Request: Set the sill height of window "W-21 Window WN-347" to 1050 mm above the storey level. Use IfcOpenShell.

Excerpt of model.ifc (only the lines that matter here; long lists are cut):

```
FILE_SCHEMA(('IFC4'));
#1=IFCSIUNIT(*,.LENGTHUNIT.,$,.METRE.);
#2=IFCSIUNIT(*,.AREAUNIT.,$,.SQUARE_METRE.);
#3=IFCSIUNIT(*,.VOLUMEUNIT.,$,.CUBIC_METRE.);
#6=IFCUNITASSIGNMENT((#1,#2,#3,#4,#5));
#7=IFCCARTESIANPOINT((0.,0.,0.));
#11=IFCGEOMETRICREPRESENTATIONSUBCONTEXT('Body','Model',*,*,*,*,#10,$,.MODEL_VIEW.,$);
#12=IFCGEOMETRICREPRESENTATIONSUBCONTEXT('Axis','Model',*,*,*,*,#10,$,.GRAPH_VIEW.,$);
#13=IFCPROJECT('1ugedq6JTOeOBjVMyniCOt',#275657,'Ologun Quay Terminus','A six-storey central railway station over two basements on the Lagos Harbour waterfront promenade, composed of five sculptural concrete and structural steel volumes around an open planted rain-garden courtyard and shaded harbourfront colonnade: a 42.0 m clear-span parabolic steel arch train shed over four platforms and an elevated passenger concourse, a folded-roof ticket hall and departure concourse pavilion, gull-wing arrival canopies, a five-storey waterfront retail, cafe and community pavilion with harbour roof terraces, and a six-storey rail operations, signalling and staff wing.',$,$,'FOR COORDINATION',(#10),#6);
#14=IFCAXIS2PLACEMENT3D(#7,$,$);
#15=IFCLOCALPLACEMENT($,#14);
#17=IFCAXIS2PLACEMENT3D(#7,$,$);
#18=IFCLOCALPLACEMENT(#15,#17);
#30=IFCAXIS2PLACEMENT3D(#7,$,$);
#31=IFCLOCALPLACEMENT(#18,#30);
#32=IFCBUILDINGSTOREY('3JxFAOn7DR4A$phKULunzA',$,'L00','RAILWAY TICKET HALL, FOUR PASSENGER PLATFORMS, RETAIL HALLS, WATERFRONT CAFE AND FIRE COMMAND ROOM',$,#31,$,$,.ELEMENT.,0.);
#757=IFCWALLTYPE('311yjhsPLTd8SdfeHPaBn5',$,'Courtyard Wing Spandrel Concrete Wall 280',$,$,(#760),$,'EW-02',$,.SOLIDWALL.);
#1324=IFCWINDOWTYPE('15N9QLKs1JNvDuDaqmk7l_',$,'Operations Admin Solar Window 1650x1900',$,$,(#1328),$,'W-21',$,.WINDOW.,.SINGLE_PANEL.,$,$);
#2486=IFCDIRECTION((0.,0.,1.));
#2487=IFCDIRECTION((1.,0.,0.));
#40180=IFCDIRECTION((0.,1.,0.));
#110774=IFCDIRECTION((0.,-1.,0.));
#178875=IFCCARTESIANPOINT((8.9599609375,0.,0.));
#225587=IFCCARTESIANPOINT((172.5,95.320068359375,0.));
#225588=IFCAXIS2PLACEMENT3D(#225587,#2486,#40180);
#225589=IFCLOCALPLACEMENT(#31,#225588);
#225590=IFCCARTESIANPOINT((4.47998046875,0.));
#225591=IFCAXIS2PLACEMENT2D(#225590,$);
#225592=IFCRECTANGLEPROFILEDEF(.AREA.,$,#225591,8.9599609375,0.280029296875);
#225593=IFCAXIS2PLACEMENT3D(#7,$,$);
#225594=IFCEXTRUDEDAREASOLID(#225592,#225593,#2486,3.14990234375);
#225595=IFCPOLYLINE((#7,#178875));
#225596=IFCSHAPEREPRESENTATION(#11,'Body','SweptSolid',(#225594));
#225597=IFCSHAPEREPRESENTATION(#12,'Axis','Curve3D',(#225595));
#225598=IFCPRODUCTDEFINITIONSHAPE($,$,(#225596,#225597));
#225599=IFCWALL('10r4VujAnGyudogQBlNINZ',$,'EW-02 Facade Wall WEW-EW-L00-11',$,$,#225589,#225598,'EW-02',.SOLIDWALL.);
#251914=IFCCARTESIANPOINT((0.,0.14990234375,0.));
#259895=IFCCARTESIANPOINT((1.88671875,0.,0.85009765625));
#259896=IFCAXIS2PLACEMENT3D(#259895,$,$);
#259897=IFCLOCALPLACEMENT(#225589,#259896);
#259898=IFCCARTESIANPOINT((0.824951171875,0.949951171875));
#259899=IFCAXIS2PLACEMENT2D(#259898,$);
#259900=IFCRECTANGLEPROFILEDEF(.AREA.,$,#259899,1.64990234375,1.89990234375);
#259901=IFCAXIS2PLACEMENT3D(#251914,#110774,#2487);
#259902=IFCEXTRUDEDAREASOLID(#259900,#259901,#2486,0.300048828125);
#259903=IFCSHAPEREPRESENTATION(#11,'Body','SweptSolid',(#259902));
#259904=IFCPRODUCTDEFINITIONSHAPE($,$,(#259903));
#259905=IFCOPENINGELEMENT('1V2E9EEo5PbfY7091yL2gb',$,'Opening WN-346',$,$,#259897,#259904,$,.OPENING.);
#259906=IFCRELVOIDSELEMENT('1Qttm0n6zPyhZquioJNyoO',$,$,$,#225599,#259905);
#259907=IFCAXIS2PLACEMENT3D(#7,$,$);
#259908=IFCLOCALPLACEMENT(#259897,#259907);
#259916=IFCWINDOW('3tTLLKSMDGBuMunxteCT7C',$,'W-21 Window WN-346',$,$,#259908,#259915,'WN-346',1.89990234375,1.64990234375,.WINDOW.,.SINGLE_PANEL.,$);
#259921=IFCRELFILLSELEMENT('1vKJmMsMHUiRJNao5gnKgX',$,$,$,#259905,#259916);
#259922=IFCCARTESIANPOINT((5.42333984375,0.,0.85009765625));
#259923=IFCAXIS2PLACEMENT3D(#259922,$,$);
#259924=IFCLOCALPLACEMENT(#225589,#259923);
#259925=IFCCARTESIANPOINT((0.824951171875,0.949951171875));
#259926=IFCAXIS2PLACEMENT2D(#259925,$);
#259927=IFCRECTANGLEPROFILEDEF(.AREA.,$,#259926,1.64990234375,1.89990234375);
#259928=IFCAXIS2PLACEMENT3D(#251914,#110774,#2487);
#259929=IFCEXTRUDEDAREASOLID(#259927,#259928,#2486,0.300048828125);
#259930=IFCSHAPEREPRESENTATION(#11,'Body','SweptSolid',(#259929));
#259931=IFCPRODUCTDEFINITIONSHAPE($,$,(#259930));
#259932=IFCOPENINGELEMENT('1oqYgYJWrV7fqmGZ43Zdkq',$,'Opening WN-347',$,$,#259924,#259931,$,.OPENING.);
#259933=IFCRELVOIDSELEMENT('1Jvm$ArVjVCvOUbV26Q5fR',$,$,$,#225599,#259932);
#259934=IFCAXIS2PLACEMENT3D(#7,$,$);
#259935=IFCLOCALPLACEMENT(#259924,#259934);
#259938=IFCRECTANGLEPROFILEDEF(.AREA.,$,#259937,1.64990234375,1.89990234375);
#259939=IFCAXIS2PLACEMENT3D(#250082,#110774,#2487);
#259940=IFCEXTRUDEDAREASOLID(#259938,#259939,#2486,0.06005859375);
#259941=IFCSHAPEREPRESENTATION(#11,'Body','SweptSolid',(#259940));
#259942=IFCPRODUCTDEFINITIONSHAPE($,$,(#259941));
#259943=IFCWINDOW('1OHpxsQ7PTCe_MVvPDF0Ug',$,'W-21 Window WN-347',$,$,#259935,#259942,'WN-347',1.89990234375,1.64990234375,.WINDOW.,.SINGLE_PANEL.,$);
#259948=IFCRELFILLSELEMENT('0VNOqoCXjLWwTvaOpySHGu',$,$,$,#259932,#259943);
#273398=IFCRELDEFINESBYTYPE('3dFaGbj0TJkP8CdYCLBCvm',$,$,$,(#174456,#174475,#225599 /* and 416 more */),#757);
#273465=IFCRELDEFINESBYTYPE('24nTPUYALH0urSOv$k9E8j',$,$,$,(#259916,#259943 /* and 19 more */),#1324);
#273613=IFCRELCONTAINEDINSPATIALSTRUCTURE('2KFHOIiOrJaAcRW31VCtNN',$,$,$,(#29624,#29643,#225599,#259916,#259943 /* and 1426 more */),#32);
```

```python
import numpy as np
import ifcopenshell
import ifcopenshell.api.geometry
import ifcopenshell.geom
import ifcopenshell.util.element
import ifcopenshell.util.placement
import ifcopenshell.util.shape
import ifcopenshell.util.unit

model = ifcopenshell.open("model.ifc")
unit_scale = ifcopenshell.util.unit.calculate_unit_scale(model)

window = model.by_guid("1OHpxsQ7PTCe_MVvPDF0Ug")
opening = window.FillsVoids[0].RelatingOpeningElement
storey = ifcopenshell.util.element.get_container(window, ifc_class="IfcBuildingStorey")
level = ifcopenshell.util.placement.get_local_placement(storey.ObjectPlacement)[2, 3]

# The opening's origin need not be at the sill, so measure its lowest point.
shape = ifcopenshell.geom.create_shape(ifcopenshell.geom.settings(), opening)
bottom = ifcopenshell.util.shape.get_shape_bottom_elevation(shape, shape.geometry) / unit_scale
dz = level + 1.05 - bottom

shift = np.array([0.0, 0.0, dz])
# The window is placed relative to its opening, so it follows when the opening moves.
matrix = ifcopenshell.util.placement.get_local_placement(opening.ObjectPlacement)
matrix[:3, 3] += shift
ifcopenshell.api.geometry.edit_object_placement(
    model, product=opening, matrix=matrix, is_si=False, should_transform_children=True
)

print(f"moved by {dz * unit_scale:+.3f} m")

model.write("model_v2.ifc")
```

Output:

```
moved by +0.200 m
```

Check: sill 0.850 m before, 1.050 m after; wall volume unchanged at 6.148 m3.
